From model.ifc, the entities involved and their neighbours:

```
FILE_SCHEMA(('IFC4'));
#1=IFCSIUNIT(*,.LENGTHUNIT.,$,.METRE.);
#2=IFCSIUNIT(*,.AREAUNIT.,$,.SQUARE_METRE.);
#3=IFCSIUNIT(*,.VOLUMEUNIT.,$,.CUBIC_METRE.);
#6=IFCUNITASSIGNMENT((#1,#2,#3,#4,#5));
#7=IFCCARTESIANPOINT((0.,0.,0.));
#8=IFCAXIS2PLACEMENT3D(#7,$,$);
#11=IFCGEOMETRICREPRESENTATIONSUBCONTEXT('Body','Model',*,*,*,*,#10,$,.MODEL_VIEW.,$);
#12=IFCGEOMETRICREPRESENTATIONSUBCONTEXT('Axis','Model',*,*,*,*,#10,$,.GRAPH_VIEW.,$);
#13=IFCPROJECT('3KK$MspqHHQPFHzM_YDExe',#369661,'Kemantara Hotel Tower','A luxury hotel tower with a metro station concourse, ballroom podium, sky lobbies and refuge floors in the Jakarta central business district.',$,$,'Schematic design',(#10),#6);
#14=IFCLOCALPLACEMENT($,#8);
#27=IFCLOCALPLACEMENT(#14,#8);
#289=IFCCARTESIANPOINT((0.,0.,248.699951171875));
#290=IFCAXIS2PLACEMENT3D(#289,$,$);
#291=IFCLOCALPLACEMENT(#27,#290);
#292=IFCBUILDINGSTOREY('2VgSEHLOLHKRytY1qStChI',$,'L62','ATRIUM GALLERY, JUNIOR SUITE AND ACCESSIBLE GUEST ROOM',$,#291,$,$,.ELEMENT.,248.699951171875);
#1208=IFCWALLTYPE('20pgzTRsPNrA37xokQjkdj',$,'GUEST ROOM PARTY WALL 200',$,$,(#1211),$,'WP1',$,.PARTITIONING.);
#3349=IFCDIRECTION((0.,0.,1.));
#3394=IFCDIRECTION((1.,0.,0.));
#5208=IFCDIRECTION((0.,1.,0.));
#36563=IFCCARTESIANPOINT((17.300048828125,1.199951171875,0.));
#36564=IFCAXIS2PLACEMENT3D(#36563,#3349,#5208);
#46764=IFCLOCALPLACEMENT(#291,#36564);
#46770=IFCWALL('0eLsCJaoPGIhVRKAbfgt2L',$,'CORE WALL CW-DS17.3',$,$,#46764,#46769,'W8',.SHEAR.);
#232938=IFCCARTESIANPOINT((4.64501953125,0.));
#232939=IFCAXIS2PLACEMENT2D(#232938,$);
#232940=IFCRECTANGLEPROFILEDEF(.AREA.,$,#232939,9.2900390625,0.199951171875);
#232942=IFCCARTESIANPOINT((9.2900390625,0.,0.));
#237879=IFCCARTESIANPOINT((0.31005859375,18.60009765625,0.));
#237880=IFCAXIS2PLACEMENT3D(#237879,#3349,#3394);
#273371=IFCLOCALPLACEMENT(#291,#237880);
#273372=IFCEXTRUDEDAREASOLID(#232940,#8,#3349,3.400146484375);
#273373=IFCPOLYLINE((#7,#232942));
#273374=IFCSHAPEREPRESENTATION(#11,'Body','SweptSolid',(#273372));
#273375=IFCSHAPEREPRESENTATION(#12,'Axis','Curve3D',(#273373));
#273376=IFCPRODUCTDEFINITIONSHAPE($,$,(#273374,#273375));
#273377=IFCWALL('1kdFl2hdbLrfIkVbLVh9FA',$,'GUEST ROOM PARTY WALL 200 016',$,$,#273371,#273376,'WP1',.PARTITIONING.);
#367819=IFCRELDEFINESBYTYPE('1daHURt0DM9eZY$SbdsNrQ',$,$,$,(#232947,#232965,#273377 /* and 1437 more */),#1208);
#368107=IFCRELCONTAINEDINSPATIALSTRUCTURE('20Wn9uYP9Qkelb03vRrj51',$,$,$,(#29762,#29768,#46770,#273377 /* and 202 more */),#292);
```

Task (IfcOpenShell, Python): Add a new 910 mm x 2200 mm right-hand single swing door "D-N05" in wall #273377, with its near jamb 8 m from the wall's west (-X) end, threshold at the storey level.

```python
import numpy as np
import ifcopenshell
import ifcopenshell.api.feature
import ifcopenshell.api.geometry
import ifcopenshell.api.root
import ifcopenshell.api.spatial
import ifcopenshell.geom
import ifcopenshell.util.element
import ifcopenshell.util.placement
import ifcopenshell.util.representation
import ifcopenshell.util.shape
import ifcopenshell.util.unit

model = ifcopenshell.open("model.ifc")
unit_scale = ifcopenshell.util.unit.calculate_unit_scale(model)
settings = ifcopenshell.geom.settings()


def volume(element):
    """Net volume in cubic metres, openings subtracted."""
    shape = ifcopenshell.geom.create_shape(settings, element)
    return ifcopenshell.util.shape.get_volume(shape.geometry)


wall = model.by_guid("1kdFl2hdbLrfIkVbLVh9FA")
storey = ifcopenshell.util.element.get_container(wall, ifc_class="IfcBuildingStorey")
context = ifcopenshell.util.representation.get_context(model, "Model", "Body", "MODEL_VIEW")
before = volume(wall)

width, height, from_end, sill = 0.91, 2.2, 8, 0.0  # metres

# The wall runs along its own X axis, and the end named is its -X end.
wall_shape = ifcopenshell.geom.create_shape(settings, wall)
x, y, z = ifcopenshell.util.shape.get_vertices(wall_shape.geometry).T
start = x.min() + from_end
face, thickness = float(y.min()), float(y.max() - y.min())
wall_matrix = ifcopenshell.util.placement.get_local_placement(wall.ObjectPlacement)
level = ifcopenshell.util.placement.get_local_placement(storey.ObjectPlacement)[2, 3]


def in_wall(x, y):
    """Placement at x, y metres in the wall's axes, at sill height."""
    matrix = wall_matrix.copy()
    matrix[:, 3] = wall_matrix @ np.array([x / unit_scale, y / unit_scale, 0.0, 1.0])
    matrix[2, 3] = level + sill / unit_scale
    return matrix


# Opening: a box that overshoots both wall faces by 50 mm.
opening = ifcopenshell.api.root.create_entity(model, ifc_class="IfcOpeningElement", predefined_type="OPENING")
box = ifcopenshell.api.geometry.add_wall_representation(
    model, context=context, length=width, height=height, thickness=thickness + 0.1
)
ifcopenshell.api.geometry.assign_representation(model, product=opening, representation=box)
ifcopenshell.api.geometry.edit_object_placement(model, product=opening, matrix=in_wall(start, face - 0.05), is_si=False)
ifcopenshell.api.feature.add_feature(model, feature=opening, element=wall)

door = ifcopenshell.api.root.create_entity(model, ifc_class="IfcDoor", name="D-N05", predefined_type="DOOR")
door.OverallWidth, door.OverallHeight = width / unit_scale, height / unit_scale
door.OperationType = "SINGLE_SWING_RIGHT"
body = ifcopenshell.api.geometry.add_door_representation(
    model,
    context=context,
    overall_width=door.OverallWidth,
    overall_height=door.OverallHeight,
    operation_type="SINGLE_SWING_RIGHT",
    lining_properties={"LiningDepth": thickness / unit_scale, "ThresholdDepth": thickness / unit_scale},
)
ifcopenshell.api.geometry.assign_representation(model, product=door, representation=body)
ifcopenshell.api.spatial.assign_container(model, products=[door], relating_structure=storey)
ifcopenshell.api.feature.add_filling(model, opening=opening, element=door)

# The lining spans the wall, so the door starts at the wall face.
ifcopenshell.api.geometry.edit_object_placement(model, product=door, matrix=in_wall(start, face), is_si=False)

after = volume(wall)

print(f"wall volume {before:.3f} -> {after:.3f} m3")

model.write("model_rev.ifc")
```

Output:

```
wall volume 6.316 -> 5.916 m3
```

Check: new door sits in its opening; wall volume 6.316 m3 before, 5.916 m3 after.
